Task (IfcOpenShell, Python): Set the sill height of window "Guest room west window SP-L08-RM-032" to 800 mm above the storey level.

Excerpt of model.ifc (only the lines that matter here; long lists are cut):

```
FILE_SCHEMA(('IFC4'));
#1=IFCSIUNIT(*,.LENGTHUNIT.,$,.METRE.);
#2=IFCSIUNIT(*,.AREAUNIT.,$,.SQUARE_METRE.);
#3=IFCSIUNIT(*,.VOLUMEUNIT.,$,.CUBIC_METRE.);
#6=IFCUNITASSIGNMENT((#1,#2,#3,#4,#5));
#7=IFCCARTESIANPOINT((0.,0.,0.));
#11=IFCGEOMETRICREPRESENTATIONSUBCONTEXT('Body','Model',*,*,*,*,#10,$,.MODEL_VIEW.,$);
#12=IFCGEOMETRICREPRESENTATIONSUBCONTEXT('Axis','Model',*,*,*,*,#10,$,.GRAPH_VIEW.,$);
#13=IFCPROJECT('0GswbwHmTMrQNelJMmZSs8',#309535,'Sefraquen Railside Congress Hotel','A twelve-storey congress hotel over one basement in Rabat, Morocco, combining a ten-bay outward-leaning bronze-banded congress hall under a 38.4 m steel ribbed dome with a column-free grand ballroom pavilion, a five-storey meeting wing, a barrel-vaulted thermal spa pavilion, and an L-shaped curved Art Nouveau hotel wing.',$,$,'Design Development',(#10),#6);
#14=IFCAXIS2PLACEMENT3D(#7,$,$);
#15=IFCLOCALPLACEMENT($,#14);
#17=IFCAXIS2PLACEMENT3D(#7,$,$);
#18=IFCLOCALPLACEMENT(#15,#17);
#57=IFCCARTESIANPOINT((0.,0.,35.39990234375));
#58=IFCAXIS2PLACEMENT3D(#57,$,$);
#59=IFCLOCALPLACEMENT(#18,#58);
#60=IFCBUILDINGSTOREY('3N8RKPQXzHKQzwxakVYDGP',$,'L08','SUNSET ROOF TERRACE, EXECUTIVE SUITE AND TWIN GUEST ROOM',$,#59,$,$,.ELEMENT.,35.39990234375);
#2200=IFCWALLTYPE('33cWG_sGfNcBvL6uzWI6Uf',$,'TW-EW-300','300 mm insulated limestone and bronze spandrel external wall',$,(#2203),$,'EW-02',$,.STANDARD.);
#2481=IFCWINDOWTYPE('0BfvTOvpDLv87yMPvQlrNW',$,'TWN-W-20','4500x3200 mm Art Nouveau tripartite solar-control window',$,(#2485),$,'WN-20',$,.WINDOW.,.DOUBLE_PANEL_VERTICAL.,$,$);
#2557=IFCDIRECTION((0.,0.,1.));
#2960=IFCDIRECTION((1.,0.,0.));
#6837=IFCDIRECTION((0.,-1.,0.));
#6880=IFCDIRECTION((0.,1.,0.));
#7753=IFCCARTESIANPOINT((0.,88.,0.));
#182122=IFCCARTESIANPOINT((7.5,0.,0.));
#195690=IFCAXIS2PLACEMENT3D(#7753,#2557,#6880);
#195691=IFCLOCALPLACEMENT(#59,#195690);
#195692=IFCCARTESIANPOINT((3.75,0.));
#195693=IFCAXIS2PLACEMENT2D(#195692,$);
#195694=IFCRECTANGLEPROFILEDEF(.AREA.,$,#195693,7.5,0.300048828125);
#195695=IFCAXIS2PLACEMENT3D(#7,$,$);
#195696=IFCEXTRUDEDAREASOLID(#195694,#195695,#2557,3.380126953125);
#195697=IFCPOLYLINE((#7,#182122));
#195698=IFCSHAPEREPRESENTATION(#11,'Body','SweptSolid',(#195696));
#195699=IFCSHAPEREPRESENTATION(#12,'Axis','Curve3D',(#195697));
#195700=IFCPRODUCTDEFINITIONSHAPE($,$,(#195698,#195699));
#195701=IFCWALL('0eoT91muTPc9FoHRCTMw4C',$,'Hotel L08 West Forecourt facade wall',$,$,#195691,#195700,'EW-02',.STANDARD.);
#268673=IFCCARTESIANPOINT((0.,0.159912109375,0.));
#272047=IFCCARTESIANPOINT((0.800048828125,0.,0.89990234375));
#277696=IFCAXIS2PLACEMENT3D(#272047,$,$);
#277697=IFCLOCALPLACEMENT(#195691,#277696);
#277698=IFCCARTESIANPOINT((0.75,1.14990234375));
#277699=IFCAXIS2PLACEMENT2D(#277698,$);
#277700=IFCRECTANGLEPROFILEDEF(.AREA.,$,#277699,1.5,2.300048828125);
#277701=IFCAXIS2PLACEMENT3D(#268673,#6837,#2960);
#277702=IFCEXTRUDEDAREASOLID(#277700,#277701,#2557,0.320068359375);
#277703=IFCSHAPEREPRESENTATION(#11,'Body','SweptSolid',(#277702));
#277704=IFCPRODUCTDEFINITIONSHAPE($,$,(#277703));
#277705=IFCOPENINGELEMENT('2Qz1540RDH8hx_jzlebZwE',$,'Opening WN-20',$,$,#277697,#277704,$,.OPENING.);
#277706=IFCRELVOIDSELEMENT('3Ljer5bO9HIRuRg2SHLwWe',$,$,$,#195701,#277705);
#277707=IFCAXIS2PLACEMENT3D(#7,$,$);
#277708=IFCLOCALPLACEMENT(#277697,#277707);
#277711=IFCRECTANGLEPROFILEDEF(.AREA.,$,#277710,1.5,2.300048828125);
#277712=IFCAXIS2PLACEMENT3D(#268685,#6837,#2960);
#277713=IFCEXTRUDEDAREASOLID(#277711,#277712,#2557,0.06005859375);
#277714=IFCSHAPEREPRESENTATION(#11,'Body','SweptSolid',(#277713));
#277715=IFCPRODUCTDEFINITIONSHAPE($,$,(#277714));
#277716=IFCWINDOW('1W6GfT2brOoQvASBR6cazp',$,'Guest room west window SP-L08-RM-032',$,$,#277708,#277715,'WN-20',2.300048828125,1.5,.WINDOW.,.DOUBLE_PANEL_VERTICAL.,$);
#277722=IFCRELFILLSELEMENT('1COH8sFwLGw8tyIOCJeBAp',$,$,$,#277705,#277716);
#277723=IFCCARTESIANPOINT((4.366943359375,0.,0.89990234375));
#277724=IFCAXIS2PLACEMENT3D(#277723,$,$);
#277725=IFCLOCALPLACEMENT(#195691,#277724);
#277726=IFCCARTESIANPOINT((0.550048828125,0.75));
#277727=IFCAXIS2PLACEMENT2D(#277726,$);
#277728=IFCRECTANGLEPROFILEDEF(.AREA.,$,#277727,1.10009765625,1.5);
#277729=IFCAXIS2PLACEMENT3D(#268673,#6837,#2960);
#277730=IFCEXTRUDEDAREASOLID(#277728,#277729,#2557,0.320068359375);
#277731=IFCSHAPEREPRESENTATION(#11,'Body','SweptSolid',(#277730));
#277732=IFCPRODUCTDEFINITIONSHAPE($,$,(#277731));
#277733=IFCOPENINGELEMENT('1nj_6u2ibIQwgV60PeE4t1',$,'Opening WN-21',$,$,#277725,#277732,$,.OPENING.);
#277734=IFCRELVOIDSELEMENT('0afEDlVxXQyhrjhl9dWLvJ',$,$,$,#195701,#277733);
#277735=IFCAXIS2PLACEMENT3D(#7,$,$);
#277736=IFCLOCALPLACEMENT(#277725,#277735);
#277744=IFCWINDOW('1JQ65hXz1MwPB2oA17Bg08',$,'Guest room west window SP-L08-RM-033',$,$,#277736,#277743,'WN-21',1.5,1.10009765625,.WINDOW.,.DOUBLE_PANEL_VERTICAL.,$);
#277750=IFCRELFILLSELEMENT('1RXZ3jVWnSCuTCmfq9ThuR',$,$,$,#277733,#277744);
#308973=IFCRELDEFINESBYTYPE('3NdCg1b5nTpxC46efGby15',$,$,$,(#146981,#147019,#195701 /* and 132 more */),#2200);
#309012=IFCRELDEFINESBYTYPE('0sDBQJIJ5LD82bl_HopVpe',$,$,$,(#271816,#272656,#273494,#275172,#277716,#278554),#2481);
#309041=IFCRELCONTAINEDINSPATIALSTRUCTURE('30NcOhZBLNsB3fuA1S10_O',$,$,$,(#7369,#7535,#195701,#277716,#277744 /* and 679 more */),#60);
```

```python
import numpy as np
import ifcopenshell
import ifcopenshell.api.geometry
import ifcopenshell.geom
import ifcopenshell.util.element
import ifcopenshell.util.placement
import ifcopenshell.util.shape
import ifcopenshell.util.unit

model = ifcopenshell.open("model.ifc")
unit_scale = ifcopenshell.util.unit.calculate_unit_scale(model)

window = model.by_id(277716)
opening = window.FillsVoids[0].RelatingOpeningElement
storey = ifcopenshell.util.element.get_container(window, ifc_class="IfcBuildingStorey")
level = ifcopenshell.util.placement.get_local_placement(storey.ObjectPlacement)[2, 3]

# The opening's origin need not be at the sill, so measure its lowest point.
shape = ifcopenshell.geom.create_shape(ifcopenshell.geom.settings(), opening)
bottom = ifcopenshell.util.shape.get_shape_bottom_elevation(shape, shape.geometry) / unit_scale
dz = level + 0.8 / unit_scale - bottom

shift = np.array([0.0, 0.0, dz])
# The window is placed relative to its opening, so it follows when the opening moves.
matrix = ifcopenshell.util.placement.get_local_placement(opening.ObjectPlacement)
matrix[:3, 3] += shift
ifcopenshell.api.geometry.edit_object_placement(
    model, product=opening, matrix=matrix, is_si=False, should_transform_children=True
)

print(f"moved by {dz * unit_scale:+.3f} m")

model.write("model_updated.ifc")
```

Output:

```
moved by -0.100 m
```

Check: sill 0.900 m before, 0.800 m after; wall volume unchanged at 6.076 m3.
